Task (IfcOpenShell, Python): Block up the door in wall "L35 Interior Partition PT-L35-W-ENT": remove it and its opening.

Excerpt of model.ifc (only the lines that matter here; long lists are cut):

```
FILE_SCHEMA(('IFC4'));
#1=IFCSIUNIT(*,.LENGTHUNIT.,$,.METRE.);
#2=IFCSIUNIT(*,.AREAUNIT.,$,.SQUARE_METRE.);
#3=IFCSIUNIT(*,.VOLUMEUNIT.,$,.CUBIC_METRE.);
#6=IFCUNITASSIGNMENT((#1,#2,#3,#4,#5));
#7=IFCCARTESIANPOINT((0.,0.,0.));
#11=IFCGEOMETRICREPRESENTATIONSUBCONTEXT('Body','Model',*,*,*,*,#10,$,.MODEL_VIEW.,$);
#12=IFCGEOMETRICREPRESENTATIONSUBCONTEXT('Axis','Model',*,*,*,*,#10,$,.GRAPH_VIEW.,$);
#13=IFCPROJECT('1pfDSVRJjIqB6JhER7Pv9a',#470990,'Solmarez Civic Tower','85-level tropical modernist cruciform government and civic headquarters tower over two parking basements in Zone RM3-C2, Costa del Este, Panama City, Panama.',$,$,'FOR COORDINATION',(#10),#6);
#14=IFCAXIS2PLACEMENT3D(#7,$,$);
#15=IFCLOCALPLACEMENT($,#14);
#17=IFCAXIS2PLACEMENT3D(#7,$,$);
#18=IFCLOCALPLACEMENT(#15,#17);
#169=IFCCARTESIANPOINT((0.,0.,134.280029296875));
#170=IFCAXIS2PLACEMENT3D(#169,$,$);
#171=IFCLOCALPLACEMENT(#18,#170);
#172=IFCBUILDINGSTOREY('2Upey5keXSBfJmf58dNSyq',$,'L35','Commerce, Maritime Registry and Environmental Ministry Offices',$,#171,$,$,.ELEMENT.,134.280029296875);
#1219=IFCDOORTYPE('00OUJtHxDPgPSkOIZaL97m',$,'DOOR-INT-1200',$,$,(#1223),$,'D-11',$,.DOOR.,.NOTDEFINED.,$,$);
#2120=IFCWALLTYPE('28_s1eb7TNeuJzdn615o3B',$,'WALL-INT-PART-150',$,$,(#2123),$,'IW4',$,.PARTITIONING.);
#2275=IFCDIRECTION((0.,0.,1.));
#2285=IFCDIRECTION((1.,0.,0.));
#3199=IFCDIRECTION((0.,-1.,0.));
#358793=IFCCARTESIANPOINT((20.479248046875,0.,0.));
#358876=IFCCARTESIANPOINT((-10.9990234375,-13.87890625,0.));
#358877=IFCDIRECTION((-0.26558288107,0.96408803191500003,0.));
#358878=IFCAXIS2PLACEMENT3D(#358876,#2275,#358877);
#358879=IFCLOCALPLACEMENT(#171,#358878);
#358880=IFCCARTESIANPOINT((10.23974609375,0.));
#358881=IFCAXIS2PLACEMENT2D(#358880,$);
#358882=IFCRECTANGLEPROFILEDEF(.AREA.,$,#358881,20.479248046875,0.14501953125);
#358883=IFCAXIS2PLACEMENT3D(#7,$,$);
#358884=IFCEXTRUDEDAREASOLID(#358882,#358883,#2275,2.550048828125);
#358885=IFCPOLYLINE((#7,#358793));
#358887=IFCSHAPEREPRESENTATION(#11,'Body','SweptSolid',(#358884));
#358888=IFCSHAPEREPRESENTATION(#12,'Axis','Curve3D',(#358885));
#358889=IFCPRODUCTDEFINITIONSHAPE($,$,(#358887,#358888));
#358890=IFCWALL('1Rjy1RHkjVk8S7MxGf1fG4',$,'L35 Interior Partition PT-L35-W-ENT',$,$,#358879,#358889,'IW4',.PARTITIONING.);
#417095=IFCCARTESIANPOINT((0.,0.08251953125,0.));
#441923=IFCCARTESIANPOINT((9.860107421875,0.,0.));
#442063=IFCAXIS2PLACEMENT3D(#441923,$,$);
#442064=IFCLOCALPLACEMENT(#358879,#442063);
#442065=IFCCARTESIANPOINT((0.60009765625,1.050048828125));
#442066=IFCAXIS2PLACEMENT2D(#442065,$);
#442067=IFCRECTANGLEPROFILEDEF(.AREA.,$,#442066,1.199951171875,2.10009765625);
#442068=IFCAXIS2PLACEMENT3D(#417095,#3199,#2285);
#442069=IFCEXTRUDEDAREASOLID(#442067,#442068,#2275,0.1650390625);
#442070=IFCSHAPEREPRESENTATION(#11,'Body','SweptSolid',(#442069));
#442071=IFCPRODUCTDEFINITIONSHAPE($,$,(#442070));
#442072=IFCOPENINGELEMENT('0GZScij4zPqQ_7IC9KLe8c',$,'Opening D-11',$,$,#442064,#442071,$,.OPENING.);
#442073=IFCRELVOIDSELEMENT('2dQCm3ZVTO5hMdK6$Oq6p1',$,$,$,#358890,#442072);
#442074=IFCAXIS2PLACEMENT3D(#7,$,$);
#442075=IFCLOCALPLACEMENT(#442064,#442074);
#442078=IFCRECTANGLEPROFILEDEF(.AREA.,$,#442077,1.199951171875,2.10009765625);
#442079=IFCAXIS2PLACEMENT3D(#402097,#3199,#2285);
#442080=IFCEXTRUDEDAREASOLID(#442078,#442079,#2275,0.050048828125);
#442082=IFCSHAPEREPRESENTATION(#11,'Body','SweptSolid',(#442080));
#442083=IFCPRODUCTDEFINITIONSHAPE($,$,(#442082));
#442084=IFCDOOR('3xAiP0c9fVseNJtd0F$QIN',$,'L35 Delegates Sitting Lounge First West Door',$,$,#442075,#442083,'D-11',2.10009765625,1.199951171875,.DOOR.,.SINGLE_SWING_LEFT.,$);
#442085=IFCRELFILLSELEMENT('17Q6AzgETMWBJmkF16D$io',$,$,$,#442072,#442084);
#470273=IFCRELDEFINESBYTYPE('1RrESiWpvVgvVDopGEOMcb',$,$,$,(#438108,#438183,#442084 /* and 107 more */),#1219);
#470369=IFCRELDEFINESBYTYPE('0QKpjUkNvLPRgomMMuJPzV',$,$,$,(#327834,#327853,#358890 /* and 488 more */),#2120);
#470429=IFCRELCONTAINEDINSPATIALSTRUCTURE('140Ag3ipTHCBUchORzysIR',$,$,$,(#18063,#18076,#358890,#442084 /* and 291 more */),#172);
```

```python
import ifcopenshell
import ifcopenshell.api.feature
import ifcopenshell.api.root
import ifcopenshell.geom
import ifcopenshell.util.shape

model = ifcopenshell.open("model.ifc")
settings = ifcopenshell.geom.settings()


def volume(element):
    """Net volume in cubic metres, openings subtracted."""
    shape = ifcopenshell.geom.create_shape(settings, element)
    return ifcopenshell.util.shape.get_volume(shape.geometry)


door = model.by_guid("3xAiP0c9fVseNJtd0F$QIN")
opening = door.FillsVoids[0].RelatingOpeningElement
wall = opening.VoidsElements[0].RelatingBuildingElement
before = volume(wall)

ifcopenshell.api.root.remove_product(model, product=door)
ifcopenshell.api.feature.remove_feature(model, feature=opening)

after = volume(wall)

print(f"wall volume {before:.3f} -> {after:.3f} m3")

model.write("model_updated.ifc")
```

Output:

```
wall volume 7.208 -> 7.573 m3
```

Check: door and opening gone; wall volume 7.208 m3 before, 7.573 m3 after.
